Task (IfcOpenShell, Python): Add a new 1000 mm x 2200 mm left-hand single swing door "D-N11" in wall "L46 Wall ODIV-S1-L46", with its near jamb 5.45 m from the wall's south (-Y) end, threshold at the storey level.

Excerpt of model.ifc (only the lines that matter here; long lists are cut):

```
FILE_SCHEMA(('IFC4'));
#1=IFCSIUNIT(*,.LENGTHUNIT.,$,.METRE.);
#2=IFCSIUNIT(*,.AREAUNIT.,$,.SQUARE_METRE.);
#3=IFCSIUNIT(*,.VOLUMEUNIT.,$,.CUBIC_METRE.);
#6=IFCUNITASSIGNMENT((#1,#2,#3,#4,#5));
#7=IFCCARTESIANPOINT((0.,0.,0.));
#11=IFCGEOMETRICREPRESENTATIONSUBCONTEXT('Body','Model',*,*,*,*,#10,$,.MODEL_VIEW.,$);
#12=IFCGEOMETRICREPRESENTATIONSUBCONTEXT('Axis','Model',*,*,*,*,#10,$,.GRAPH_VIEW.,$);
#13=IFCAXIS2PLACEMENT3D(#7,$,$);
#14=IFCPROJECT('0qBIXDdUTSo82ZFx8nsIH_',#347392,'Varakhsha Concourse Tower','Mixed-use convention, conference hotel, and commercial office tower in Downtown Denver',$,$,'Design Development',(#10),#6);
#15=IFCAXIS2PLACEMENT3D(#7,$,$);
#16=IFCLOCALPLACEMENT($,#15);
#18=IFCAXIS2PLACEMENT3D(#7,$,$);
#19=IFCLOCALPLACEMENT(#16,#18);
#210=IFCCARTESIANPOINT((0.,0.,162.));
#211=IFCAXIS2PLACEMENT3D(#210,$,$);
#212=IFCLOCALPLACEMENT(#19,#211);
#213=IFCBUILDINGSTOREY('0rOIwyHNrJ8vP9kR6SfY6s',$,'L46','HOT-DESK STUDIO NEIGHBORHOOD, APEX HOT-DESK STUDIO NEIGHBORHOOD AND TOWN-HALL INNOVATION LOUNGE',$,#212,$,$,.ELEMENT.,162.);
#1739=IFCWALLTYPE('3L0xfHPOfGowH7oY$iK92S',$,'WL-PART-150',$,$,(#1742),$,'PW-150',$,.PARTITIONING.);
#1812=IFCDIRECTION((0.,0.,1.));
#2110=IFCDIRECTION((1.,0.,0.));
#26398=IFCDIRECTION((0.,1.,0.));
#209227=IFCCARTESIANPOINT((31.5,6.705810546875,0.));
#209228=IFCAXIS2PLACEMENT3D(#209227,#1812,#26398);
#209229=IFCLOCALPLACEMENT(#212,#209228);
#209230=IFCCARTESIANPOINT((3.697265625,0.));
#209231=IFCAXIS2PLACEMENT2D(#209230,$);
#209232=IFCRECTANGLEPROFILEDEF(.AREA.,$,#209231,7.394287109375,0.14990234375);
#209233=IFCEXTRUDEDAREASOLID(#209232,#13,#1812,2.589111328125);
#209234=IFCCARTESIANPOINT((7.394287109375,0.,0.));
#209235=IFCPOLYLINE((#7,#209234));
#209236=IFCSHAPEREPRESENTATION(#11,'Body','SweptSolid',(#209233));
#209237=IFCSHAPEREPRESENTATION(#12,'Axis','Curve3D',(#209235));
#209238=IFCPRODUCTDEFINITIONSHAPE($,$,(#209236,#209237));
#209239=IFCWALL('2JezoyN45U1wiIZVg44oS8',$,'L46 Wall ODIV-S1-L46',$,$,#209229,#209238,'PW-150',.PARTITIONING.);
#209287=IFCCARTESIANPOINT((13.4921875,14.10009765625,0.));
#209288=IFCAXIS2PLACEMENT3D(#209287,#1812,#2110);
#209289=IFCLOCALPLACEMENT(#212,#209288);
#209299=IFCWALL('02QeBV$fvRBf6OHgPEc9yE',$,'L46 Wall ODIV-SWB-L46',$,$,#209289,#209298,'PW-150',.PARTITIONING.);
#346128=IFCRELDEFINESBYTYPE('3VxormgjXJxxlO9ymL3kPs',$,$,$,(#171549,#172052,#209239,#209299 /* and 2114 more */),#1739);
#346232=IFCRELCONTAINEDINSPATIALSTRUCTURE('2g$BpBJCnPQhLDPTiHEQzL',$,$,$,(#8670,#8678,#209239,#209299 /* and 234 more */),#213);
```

```python
import numpy as np
import ifcopenshell
import ifcopenshell.api.feature
import ifcopenshell.api.geometry
import ifcopenshell.api.root
import ifcopenshell.api.spatial
import ifcopenshell.geom
import ifcopenshell.util.element
import ifcopenshell.util.placement
import ifcopenshell.util.representation
import ifcopenshell.util.shape
import ifcopenshell.util.unit

model = ifcopenshell.open("model.ifc")
unit_scale = ifcopenshell.util.unit.calculate_unit_scale(model)
settings = ifcopenshell.geom.settings()


def volume(element):
    """Net volume in cubic metres, openings subtracted."""
    shape = ifcopenshell.geom.create_shape(settings, element)
    return ifcopenshell.util.shape.get_volume(shape.geometry)


wall = model.by_guid("2JezoyN45U1wiIZVg44oS8")
storey = ifcopenshell.util.element.get_container(wall, ifc_class="IfcBuildingStorey")
context = ifcopenshell.util.representation.get_context(model, "Model", "Body", "MODEL_VIEW")
before = volume(wall)

width, height, from_end, sill = 1, 2.2, 5.45, 0.0  # metres

# The wall runs along its own X axis, and the end named is its -X end.
wall_shape = ifcopenshell.geom.create_shape(settings, wall)
x, y, z = ifcopenshell.util.shape.get_vertices(wall_shape.geometry).T
start = x.min() + from_end
face, thickness = float(y.min()), float(y.max() - y.min())
wall_matrix = ifcopenshell.util.placement.get_local_placement(wall.ObjectPlacement)
level = ifcopenshell.util.placement.get_local_placement(storey.ObjectPlacement)[2, 3]


def in_wall(x, y):
    """Placement at x, y metres in the wall's axes, at sill height."""
    matrix = wall_matrix.copy()
    matrix[:, 3] = wall_matrix @ np.array([x / unit_scale, y / unit_scale, 0.0, 1.0])
    matrix[2, 3] = level + sill / unit_scale
    return matrix


# Opening: a box that overshoots both wall faces by 50 mm.
opening = ifcopenshell.api.root.create_entity(model, ifc_class="IfcOpeningElement", predefined_type="OPENING")
box = ifcopenshell.api.geometry.add_wall_representation(
    model, context=context, length=width, height=height, thickness=thickness + 0.1
)
ifcopenshell.api.geometry.assign_representation(model, product=opening, representation=box)
ifcopenshell.api.geometry.edit_object_placement(model, product=opening, matrix=in_wall(start, face - 0.05), is_si=False)
ifcopenshell.api.feature.add_feature(model, feature=opening, element=wall)

door = ifcopenshell.api.root.create_entity(model, ifc_class="IfcDoor", name="D-N11", predefined_type="DOOR")
door.OverallWidth, door.OverallHeight = width / unit_scale, height / unit_scale
door.OperationType = "SINGLE_SWING_LEFT"
body = ifcopenshell.api.geometry.add_door_representation(
    model,
    context=context,
    overall_width=door.OverallWidth,
    overall_height=door.OverallHeight,
    operation_type="SINGLE_SWING_LEFT",
    lining_properties={"LiningDepth": thickness / unit_scale, "ThresholdDepth": thickness / unit_scale},
)
ifcopenshell.api.geometry.assign_representation(model, product=door, representation=body)
ifcopenshell.api.spatial.assign_container(model, products=[door], relating_structure=storey)
ifcopenshell.api.feature.add_filling(model, opening=opening, element=door)

# The lining spans the wall, so the door starts at the wall face.
ifcopenshell.api.geometry.edit_object_placement(model, product=door, matrix=in_wall(start, face), is_si=False)

after = volume(wall)

print(f"wall volume {before:.3f} -> {after:.3f} m3")

model.write("model_edited.ifc")
```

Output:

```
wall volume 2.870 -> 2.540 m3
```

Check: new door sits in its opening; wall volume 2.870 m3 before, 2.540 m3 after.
